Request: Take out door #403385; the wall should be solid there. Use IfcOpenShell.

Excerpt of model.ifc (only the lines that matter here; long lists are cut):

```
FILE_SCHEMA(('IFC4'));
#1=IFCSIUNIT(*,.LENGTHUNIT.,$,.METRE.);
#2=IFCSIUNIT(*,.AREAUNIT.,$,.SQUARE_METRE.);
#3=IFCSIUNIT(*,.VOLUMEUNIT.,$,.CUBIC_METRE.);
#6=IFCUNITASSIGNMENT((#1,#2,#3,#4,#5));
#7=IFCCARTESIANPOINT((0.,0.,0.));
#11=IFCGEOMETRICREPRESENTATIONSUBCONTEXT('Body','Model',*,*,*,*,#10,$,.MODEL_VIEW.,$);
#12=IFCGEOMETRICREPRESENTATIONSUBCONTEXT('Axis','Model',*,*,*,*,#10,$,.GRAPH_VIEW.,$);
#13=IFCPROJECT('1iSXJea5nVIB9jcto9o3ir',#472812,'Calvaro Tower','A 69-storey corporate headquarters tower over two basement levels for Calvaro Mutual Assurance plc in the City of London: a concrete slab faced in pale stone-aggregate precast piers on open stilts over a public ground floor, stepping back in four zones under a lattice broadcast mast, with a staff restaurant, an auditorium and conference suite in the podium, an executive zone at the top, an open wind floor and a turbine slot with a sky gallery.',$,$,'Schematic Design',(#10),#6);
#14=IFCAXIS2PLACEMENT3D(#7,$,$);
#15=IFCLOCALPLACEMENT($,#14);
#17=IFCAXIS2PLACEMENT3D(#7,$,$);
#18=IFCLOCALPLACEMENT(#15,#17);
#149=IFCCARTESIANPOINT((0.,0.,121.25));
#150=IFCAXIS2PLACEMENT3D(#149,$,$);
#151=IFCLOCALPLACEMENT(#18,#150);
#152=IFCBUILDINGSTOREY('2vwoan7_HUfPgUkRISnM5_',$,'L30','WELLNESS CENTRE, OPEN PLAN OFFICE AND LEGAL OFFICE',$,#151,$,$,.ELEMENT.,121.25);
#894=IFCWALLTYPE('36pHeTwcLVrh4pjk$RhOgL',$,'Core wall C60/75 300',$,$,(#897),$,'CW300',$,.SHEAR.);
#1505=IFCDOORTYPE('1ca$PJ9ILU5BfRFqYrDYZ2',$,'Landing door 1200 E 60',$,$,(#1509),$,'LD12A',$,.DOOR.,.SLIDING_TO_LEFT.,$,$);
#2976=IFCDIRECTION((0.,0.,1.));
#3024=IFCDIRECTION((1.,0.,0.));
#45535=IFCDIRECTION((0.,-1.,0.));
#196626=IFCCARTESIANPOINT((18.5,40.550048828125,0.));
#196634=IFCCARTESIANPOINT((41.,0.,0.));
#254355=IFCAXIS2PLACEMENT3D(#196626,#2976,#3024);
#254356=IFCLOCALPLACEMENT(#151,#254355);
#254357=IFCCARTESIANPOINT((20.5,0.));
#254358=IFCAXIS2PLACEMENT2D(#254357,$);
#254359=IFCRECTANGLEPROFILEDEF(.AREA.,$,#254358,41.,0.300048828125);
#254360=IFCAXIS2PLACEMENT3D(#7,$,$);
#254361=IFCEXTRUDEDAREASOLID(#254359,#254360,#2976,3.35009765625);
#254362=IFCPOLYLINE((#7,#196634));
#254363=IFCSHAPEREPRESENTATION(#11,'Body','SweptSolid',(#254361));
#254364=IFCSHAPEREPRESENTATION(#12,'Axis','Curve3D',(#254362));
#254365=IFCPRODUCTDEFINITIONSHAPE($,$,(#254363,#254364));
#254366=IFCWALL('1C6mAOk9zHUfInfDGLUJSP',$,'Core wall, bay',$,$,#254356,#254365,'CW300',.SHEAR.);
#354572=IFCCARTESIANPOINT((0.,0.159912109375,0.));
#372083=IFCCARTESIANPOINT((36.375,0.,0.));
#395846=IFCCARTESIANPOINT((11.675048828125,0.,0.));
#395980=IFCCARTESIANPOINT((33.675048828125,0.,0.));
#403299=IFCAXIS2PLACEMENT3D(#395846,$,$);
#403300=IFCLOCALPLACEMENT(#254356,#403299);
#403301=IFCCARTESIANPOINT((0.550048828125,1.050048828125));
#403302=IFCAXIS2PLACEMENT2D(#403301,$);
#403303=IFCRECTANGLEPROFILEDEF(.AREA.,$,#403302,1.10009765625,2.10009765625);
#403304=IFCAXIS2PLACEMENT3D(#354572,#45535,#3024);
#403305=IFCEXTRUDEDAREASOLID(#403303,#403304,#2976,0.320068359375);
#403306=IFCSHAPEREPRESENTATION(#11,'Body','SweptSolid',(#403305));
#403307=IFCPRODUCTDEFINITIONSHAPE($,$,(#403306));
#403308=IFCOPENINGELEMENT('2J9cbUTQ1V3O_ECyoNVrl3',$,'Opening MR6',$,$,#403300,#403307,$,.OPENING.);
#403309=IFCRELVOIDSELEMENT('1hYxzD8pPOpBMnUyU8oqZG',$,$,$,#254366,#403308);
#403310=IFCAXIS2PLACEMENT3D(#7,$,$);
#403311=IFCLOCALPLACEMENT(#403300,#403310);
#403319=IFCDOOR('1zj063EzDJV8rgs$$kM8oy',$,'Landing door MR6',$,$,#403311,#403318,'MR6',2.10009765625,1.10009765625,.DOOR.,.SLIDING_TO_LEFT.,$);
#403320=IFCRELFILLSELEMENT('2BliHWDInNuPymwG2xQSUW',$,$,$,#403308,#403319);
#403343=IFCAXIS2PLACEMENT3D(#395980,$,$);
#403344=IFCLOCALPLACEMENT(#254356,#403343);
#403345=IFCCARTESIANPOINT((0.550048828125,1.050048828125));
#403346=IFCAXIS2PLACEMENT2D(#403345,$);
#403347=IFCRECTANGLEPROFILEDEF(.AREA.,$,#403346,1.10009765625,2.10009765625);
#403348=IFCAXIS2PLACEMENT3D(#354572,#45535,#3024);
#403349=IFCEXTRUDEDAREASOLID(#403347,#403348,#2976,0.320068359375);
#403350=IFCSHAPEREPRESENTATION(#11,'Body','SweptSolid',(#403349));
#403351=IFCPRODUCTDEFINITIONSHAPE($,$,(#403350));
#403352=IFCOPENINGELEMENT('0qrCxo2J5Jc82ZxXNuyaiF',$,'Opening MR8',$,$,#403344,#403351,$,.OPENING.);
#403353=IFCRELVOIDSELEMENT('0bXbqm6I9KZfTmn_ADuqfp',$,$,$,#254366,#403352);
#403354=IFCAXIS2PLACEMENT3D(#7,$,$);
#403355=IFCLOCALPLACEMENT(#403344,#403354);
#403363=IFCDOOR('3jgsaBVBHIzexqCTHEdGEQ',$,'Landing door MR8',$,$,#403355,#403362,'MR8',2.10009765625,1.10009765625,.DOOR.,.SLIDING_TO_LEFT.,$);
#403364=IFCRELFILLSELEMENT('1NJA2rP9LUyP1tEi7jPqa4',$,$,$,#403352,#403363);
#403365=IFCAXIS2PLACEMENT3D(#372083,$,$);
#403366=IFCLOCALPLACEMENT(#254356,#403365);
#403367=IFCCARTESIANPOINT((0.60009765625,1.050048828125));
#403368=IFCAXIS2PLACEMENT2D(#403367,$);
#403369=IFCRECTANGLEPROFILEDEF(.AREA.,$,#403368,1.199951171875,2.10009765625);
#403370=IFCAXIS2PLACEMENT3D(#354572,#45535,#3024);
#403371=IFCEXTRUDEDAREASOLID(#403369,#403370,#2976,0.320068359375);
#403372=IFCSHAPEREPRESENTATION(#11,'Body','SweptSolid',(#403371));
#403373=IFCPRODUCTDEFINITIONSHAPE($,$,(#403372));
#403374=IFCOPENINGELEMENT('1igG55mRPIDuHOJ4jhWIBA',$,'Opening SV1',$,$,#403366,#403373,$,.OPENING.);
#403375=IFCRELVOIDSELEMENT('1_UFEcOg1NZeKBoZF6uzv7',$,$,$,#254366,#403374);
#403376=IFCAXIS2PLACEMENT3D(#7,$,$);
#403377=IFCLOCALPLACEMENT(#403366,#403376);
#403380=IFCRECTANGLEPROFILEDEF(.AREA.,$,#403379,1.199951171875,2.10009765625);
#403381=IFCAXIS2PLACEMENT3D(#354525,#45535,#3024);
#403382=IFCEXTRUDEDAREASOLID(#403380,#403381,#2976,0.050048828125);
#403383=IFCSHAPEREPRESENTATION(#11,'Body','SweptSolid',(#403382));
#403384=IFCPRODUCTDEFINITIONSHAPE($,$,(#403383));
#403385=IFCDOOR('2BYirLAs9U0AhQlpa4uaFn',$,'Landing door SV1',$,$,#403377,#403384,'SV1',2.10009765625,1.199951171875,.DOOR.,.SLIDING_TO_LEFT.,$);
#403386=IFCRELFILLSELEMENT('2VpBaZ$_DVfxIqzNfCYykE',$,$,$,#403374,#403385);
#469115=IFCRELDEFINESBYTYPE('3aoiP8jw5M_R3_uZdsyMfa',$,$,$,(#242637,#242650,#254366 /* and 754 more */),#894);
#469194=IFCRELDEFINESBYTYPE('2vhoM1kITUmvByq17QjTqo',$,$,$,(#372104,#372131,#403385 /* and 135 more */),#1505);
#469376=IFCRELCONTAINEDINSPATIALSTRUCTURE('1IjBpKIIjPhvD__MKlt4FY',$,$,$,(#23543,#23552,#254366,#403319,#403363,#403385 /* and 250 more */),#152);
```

```python
import ifcopenshell
import ifcopenshell.api.feature
import ifcopenshell.api.root
import ifcopenshell.geom
import ifcopenshell.util.shape

model = ifcopenshell.open("model.ifc")
settings = ifcopenshell.geom.settings()


def volume(element):
    """Net volume in cubic metres, openings subtracted."""
    shape = ifcopenshell.geom.create_shape(settings, element)
    return ifcopenshell.util.shape.get_volume(shape.geometry)


door = model.by_id(403385)
opening = door.FillsVoids[0].RelatingOpeningElement
wall = opening.VoidsElements[0].RelatingBuildingElement
before = volume(wall)

ifcopenshell.api.root.remove_product(model, product=door)
ifcopenshell.api.feature.remove_feature(model, feature=opening)

after = volume(wall)

print(f"wall volume {before:.3f} -> {after:.3f} m3")

model.write("model_edited.ifc")
```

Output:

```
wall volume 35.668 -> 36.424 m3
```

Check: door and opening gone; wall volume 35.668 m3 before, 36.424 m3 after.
